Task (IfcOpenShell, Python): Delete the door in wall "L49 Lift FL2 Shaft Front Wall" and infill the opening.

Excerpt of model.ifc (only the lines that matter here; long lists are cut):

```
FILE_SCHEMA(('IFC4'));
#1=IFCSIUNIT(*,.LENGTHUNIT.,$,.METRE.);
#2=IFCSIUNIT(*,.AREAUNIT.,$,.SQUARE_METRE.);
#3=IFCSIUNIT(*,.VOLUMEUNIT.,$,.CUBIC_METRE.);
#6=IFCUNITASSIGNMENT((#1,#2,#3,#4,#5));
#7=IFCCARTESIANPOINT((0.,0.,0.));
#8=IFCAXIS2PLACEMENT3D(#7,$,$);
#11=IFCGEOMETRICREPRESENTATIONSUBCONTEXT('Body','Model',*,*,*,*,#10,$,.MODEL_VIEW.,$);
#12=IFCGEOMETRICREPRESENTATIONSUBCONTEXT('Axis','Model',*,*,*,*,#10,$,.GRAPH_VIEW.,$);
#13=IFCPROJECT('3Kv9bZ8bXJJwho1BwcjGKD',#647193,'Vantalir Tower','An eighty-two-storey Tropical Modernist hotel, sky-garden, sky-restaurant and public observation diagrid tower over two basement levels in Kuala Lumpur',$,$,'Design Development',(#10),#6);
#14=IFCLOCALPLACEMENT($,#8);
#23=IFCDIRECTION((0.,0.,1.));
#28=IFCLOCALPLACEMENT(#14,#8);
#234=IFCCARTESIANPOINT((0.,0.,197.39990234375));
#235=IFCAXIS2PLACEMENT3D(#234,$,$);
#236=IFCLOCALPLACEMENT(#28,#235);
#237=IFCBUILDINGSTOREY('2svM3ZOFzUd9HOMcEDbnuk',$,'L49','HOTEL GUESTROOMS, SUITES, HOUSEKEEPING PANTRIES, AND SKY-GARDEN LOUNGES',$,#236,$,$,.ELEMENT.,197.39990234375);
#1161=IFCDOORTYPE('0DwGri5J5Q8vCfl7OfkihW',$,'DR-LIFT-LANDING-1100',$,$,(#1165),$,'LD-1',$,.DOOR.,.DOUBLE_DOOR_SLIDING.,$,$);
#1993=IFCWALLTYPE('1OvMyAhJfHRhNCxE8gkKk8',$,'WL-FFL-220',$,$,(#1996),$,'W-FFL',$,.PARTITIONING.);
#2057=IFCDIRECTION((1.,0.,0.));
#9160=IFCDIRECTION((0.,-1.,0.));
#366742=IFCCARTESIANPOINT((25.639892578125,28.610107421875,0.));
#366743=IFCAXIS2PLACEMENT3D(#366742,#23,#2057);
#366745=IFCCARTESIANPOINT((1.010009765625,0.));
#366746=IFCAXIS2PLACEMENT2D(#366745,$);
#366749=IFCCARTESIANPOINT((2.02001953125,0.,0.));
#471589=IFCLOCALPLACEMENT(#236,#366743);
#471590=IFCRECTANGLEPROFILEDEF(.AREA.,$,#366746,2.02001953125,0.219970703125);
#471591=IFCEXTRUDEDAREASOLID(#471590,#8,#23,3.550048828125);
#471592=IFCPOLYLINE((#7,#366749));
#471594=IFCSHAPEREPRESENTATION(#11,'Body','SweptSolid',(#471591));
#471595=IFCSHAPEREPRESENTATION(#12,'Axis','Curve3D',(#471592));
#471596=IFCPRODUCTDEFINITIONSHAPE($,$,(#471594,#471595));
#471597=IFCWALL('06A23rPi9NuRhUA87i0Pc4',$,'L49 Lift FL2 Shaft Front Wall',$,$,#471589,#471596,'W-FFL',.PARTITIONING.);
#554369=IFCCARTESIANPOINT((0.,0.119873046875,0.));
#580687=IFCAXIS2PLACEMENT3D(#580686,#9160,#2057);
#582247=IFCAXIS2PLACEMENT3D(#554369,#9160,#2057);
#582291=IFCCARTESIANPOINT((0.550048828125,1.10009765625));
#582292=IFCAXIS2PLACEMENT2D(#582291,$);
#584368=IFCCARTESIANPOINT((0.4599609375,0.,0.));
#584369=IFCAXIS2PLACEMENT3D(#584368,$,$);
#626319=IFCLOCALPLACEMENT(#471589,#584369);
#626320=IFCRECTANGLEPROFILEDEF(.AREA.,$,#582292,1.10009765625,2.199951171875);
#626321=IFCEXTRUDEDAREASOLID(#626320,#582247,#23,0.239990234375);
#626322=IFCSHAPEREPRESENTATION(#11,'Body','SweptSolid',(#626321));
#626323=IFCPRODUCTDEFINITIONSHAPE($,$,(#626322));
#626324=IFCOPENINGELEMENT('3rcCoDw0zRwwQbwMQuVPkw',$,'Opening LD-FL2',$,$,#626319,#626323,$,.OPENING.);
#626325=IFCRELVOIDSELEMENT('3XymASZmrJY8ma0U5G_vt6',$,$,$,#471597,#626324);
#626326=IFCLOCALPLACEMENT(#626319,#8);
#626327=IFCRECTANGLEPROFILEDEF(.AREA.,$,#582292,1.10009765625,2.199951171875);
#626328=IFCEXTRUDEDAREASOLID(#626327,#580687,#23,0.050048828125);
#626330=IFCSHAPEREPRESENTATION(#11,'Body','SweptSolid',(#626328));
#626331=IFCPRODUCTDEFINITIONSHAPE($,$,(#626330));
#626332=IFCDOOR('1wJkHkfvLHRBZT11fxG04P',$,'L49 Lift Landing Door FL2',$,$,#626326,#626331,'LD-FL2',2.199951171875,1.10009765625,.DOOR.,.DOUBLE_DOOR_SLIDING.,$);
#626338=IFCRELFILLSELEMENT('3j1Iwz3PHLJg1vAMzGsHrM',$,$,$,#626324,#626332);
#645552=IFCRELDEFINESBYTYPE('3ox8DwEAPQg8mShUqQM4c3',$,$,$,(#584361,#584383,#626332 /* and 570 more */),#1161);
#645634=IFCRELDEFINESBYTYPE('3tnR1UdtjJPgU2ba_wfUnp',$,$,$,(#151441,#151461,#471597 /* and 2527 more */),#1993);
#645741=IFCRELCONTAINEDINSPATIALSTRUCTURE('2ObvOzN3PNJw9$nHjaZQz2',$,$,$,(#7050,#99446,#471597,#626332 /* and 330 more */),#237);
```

```python
import ifcopenshell
import ifcopenshell.api.feature
import ifcopenshell.api.root
import ifcopenshell.geom
import ifcopenshell.util.shape

model = ifcopenshell.open("model.ifc")
settings = ifcopenshell.geom.settings()


def volume(element):
    """Net volume in cubic metres, openings subtracted."""
    shape = ifcopenshell.geom.create_shape(settings, element)
    return ifcopenshell.util.shape.get_volume(shape.geometry)


door = model.by_id(626332)
opening = door.FillsVoids[0].RelatingOpeningElement
wall = opening.VoidsElements[0].RelatingBuildingElement
before = volume(wall)

ifcopenshell.api.root.remove_product(model, product=door)
ifcopenshell.api.feature.remove_feature(model, feature=opening)

after = volume(wall)

print(f"wall volume {before:.3f} -> {after:.3f} m3")

model.write("model_v2.ifc")
```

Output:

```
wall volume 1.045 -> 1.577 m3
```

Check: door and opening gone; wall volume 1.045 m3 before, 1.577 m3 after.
